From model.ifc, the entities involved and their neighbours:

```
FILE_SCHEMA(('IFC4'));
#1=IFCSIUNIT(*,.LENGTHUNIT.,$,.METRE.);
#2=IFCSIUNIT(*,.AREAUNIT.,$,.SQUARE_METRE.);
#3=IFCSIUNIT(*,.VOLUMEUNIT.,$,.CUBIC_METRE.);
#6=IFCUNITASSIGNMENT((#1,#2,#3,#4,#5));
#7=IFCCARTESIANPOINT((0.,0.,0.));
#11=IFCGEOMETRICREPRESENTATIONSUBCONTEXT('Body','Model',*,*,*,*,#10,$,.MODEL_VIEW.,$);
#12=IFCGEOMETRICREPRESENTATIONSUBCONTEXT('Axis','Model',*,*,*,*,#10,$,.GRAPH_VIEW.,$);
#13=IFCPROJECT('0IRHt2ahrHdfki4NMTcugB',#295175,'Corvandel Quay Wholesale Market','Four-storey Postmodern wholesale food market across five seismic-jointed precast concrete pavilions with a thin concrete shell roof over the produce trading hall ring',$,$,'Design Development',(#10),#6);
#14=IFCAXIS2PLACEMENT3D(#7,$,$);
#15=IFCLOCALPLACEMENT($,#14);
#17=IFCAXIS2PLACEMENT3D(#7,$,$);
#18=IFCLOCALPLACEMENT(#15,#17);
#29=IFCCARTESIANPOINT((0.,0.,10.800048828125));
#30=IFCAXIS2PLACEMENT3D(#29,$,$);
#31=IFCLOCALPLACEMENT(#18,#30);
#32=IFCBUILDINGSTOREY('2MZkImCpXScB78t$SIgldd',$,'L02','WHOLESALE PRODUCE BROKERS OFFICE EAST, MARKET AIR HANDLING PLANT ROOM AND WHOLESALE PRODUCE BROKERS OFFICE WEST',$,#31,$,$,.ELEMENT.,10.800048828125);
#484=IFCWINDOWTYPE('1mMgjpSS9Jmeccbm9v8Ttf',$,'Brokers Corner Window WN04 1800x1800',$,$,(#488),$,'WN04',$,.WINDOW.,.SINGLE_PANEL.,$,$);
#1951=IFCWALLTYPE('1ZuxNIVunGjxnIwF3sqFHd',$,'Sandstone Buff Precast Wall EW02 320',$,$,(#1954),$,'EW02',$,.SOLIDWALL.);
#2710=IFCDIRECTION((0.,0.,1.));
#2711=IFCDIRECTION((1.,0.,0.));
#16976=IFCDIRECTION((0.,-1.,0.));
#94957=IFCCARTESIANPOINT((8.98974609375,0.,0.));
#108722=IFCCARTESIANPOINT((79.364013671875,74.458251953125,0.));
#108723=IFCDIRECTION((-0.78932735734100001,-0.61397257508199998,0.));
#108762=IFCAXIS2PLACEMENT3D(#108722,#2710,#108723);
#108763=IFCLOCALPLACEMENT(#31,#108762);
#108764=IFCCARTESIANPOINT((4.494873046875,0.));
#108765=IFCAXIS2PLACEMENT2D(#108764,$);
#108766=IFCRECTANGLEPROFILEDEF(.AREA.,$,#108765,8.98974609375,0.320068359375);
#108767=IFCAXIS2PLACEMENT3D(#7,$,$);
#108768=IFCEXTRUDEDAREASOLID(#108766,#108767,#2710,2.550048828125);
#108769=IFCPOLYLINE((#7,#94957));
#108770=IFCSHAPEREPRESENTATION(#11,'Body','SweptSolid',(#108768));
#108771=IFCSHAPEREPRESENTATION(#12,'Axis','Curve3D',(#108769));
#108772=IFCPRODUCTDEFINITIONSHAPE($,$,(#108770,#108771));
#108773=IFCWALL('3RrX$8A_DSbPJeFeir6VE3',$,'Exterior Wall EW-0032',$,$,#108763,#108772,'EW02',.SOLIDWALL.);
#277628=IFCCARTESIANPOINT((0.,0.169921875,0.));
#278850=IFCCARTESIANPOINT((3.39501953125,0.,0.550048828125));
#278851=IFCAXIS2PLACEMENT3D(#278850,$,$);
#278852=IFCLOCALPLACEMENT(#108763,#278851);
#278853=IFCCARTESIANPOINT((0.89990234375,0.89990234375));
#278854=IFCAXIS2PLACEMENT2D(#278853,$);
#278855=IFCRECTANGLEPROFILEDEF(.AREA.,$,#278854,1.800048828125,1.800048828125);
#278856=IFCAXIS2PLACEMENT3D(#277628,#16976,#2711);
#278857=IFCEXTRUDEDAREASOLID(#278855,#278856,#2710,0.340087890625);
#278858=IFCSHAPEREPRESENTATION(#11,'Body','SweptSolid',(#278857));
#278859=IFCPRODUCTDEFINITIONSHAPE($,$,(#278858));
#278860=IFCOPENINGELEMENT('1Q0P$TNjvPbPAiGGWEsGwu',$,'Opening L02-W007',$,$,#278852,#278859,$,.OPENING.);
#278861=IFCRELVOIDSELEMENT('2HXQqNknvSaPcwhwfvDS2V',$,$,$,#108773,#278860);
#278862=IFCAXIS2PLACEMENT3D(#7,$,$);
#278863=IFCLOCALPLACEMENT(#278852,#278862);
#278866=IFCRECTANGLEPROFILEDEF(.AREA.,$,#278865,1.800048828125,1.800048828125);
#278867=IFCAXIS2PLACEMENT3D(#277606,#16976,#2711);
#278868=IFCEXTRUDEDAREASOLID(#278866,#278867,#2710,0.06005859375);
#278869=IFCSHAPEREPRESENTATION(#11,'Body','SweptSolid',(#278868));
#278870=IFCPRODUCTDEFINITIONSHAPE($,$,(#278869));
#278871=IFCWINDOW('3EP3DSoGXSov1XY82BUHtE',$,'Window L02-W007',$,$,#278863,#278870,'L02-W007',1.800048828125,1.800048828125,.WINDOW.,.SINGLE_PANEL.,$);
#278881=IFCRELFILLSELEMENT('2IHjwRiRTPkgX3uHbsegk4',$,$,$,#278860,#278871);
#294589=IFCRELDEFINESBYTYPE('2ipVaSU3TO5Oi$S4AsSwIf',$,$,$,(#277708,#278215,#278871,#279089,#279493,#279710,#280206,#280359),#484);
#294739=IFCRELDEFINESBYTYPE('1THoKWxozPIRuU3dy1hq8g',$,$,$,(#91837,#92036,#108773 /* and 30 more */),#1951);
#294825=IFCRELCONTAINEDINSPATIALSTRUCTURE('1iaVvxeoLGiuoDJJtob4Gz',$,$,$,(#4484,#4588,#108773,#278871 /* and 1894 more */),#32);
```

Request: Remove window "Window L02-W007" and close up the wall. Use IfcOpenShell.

```python
import ifcopenshell
import ifcopenshell.api.feature
import ifcopenshell.api.root
import ifcopenshell.geom
import ifcopenshell.util.shape

model = ifcopenshell.open("model.ifc")
settings = ifcopenshell.geom.settings()


def volume(element):
    """Net volume in cubic metres, openings subtracted."""
    shape = ifcopenshell.geom.create_shape(settings, element)
    return ifcopenshell.util.shape.get_volume(shape.geometry)


window = model.by_guid("3EP3DSoGXSov1XY82BUHtE")
opening = window.FillsVoids[0].RelatingOpeningElement
wall = opening.VoidsElements[0].RelatingBuildingElement
before = volume(wall)

ifcopenshell.api.root.remove_product(model, product=window)
ifcopenshell.api.feature.remove_feature(model, feature=opening)

after = volume(wall)

print(f"wall volume {before:.3f} -> {after:.3f} m3")

model.write("model_edited.ifc")
```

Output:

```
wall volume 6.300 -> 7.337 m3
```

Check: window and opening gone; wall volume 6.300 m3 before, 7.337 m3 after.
